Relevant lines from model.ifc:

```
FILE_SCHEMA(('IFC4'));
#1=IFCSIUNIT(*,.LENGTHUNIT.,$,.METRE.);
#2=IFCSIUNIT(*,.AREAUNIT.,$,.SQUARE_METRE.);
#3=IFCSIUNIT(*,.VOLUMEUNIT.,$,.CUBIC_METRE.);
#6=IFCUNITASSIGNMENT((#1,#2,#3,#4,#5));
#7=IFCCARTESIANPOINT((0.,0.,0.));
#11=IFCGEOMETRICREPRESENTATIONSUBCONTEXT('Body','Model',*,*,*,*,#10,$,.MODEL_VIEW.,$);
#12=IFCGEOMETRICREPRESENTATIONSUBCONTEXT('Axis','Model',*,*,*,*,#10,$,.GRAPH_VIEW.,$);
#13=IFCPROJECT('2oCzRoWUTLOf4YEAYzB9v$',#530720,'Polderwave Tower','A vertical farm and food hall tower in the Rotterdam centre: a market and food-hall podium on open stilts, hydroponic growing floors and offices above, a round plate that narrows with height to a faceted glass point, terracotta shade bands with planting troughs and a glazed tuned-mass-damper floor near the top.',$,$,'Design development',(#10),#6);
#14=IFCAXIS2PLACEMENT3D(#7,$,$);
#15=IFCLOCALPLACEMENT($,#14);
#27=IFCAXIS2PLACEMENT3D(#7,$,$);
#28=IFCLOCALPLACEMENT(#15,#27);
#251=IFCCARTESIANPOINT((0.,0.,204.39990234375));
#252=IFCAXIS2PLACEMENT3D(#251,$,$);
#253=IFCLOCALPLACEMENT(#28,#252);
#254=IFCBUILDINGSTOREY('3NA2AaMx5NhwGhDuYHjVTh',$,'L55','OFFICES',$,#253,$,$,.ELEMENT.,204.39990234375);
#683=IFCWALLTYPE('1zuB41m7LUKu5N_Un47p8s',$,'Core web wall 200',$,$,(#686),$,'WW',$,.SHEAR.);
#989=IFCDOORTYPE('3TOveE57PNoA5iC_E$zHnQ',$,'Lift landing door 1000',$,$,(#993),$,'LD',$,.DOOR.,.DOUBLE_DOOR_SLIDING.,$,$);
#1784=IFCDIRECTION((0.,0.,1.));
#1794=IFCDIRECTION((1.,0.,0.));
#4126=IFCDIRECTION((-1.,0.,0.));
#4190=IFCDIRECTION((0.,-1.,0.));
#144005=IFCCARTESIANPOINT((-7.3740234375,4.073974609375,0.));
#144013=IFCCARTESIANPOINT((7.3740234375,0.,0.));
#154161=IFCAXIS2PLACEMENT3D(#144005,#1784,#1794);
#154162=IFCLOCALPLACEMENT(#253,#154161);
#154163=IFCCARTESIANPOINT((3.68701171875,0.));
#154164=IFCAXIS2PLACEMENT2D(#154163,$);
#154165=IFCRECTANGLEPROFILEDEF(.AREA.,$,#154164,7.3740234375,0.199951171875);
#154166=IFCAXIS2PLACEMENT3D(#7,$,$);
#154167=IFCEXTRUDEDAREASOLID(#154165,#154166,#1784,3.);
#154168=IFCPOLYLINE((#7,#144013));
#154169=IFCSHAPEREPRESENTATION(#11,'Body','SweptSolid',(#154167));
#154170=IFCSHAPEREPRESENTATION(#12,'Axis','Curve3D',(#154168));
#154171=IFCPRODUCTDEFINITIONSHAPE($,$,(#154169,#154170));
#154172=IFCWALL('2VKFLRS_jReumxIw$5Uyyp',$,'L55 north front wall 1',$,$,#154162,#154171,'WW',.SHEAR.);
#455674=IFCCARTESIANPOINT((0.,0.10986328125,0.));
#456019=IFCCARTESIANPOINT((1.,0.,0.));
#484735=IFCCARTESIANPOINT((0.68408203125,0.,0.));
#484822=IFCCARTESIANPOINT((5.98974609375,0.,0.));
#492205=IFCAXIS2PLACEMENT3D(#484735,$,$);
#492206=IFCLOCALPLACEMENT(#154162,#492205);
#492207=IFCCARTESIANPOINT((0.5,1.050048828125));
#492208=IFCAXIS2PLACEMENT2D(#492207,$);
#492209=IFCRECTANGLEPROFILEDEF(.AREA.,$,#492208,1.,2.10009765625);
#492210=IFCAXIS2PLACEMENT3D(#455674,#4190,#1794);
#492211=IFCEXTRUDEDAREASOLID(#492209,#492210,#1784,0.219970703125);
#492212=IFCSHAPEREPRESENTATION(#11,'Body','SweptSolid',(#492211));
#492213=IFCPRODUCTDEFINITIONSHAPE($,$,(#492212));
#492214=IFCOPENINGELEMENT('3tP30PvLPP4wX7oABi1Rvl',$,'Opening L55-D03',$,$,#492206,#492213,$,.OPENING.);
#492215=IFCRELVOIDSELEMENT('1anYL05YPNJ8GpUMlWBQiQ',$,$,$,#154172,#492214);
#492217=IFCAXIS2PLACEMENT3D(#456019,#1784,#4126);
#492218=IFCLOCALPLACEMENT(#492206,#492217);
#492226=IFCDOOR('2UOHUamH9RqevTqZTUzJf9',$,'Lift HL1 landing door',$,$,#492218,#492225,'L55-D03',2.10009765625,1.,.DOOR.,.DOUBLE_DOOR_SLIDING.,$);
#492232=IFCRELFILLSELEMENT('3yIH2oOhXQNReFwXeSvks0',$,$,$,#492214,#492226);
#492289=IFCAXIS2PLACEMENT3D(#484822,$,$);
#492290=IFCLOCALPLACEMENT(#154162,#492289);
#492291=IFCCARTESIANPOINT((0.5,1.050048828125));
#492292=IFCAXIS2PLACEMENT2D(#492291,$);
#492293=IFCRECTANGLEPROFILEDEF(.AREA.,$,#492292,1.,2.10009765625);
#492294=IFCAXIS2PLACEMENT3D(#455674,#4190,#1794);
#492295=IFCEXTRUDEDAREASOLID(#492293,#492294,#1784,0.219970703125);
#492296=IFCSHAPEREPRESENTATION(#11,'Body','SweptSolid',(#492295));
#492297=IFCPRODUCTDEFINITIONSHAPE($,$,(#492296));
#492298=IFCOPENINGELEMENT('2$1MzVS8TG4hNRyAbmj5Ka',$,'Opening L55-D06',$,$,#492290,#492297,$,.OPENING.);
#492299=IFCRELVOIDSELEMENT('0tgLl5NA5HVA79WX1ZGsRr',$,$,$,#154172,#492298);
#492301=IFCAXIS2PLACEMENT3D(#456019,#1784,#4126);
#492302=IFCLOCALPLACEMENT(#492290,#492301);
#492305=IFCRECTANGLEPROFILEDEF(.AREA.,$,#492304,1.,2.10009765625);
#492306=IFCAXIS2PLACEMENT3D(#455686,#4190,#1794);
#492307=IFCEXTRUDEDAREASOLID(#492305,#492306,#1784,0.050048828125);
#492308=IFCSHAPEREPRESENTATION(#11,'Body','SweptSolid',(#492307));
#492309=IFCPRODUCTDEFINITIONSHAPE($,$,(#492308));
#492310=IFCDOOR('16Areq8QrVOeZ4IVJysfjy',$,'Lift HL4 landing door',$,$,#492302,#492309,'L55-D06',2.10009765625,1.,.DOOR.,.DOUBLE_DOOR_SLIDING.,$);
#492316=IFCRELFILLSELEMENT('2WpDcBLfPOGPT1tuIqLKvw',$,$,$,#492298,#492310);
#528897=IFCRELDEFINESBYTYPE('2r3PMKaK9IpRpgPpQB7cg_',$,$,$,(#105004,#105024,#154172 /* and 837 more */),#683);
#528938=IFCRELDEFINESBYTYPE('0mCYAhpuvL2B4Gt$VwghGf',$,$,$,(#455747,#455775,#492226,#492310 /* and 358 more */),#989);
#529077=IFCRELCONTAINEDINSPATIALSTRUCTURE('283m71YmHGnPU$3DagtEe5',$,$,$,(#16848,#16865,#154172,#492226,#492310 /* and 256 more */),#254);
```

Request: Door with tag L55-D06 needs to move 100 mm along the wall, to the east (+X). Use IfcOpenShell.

```python
import ifcopenshell
import ifcopenshell.api.geometry
import ifcopenshell.util.placement
import ifcopenshell.util.unit

model = ifcopenshell.open("model.ifc")
unit_scale = ifcopenshell.util.unit.calculate_unit_scale(model)

door = model.by_guid("16Areq8QrVOeZ4IVJysfjy")
opening = door.FillsVoids[0].RelatingOpeningElement
wall = opening.VoidsElements[0].RelatingBuildingElement

wall_matrix = ifcopenshell.util.placement.get_local_placement(wall.ObjectPlacement)
shift = wall_matrix[:3, 0] * 0.1 / unit_scale
before = ifcopenshell.util.placement.get_local_placement(door.ObjectPlacement)[:3, 3].copy()

# The door is placed relative to its opening, so it follows when the opening moves.
matrix = ifcopenshell.util.placement.get_local_placement(opening.ObjectPlacement)
matrix[:3, 3] += shift
ifcopenshell.api.geometry.edit_object_placement(
    model, product=opening, matrix=matrix, is_si=False, should_transform_children=True
)

after = ifcopenshell.util.placement.get_local_placement(door.ObjectPlacement)[:3, 3]
print("door moved by", (after - before).round(3) + 0.0)

model.write("model_updated.ifc")
```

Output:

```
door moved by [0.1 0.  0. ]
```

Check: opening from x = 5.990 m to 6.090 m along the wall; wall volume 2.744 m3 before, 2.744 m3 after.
